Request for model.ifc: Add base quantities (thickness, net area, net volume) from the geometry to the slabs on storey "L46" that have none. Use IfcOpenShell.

First a look at what the model holds.

```python
import ifcopenshell
import ifcopenshell.util.element
import ifcopenshell.util.unit

model = ifcopenshell.open("model.ifc")
print(model.schema)
for unit_type in ("LENGTHUNIT", "AREAUNIT", "VOLUMEUNIT"):
    print(unit_type, ifcopenshell.util.unit.calculate_unit_scale(model, unit_type))
storey = next(s for s in model.by_type("IfcBuildingStorey") if s.Name == "L46")
slabs = [e for e in ifcopenshell.util.element.get_decomposition(storey) if e.is_a("IfcSlab")]
for e in sorted(slabs, key=lambda e: e.id()):
    print(e.id(), e.is_a(), e.Name, list(ifcopenshell.util.element.get_psets(e, qtos_only=True)), sep=" | ")
```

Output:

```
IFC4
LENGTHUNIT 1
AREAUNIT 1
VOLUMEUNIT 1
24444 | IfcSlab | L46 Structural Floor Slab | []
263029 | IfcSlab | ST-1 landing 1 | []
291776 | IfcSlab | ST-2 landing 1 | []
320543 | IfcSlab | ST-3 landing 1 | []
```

```python
import ifcopenshell
import ifcopenshell.api.pset
import ifcopenshell.geom
import ifcopenshell.util.element
import ifcopenshell.util.shape
import ifcopenshell.util.unit

model = ifcopenshell.open("model.ifc")
unit_scale = ifcopenshell.util.unit.calculate_unit_scale(model)
area_scale = ifcopenshell.util.unit.calculate_unit_scale(model, "AREAUNIT")
volume_scale = ifcopenshell.util.unit.calculate_unit_scale(model, "VOLUMEUNIT")
settings = ifcopenshell.geom.settings()

storey = next(s for s in model.by_type("IfcBuildingStorey") if s.Name == "L46")
slabs = [e for e in ifcopenshell.util.element.get_decomposition(storey) if e.is_a("IfcSlab")]

for e in sorted(slabs, key=lambda e: e.id()):
    if ifcopenshell.util.element.get_psets(e, qtos_only=True, should_inherit=False):
        continue
    # Geometry comes back in metres, in the element's own axes.
    shape = ifcopenshell.geom.create_shape(settings, e)
    values = {
        "Width": ifcopenshell.util.shape.get_z(shape.geometry) / unit_scale,
        "NetArea": ifcopenshell.util.shape.get_footprint_area(shape.geometry) / area_scale,
        "NetVolume": ifcopenshell.util.shape.get_volume(shape.geometry) / volume_scale,
    }
    qto = ifcopenshell.api.pset.add_qto(model, product=e, name="Qto_SlabBaseQuantities")
    ifcopenshell.api.pset.edit_qto(model, qto=qto, properties=values)
    print(e.id(), {k: round(v, 3) for k, v in values.items()})

model.write("model_rev.ifc")
```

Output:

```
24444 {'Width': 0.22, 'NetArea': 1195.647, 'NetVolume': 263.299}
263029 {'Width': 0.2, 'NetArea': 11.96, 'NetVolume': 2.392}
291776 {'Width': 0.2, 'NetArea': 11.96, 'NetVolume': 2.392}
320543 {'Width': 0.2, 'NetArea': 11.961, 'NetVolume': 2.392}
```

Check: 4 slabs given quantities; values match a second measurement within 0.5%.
